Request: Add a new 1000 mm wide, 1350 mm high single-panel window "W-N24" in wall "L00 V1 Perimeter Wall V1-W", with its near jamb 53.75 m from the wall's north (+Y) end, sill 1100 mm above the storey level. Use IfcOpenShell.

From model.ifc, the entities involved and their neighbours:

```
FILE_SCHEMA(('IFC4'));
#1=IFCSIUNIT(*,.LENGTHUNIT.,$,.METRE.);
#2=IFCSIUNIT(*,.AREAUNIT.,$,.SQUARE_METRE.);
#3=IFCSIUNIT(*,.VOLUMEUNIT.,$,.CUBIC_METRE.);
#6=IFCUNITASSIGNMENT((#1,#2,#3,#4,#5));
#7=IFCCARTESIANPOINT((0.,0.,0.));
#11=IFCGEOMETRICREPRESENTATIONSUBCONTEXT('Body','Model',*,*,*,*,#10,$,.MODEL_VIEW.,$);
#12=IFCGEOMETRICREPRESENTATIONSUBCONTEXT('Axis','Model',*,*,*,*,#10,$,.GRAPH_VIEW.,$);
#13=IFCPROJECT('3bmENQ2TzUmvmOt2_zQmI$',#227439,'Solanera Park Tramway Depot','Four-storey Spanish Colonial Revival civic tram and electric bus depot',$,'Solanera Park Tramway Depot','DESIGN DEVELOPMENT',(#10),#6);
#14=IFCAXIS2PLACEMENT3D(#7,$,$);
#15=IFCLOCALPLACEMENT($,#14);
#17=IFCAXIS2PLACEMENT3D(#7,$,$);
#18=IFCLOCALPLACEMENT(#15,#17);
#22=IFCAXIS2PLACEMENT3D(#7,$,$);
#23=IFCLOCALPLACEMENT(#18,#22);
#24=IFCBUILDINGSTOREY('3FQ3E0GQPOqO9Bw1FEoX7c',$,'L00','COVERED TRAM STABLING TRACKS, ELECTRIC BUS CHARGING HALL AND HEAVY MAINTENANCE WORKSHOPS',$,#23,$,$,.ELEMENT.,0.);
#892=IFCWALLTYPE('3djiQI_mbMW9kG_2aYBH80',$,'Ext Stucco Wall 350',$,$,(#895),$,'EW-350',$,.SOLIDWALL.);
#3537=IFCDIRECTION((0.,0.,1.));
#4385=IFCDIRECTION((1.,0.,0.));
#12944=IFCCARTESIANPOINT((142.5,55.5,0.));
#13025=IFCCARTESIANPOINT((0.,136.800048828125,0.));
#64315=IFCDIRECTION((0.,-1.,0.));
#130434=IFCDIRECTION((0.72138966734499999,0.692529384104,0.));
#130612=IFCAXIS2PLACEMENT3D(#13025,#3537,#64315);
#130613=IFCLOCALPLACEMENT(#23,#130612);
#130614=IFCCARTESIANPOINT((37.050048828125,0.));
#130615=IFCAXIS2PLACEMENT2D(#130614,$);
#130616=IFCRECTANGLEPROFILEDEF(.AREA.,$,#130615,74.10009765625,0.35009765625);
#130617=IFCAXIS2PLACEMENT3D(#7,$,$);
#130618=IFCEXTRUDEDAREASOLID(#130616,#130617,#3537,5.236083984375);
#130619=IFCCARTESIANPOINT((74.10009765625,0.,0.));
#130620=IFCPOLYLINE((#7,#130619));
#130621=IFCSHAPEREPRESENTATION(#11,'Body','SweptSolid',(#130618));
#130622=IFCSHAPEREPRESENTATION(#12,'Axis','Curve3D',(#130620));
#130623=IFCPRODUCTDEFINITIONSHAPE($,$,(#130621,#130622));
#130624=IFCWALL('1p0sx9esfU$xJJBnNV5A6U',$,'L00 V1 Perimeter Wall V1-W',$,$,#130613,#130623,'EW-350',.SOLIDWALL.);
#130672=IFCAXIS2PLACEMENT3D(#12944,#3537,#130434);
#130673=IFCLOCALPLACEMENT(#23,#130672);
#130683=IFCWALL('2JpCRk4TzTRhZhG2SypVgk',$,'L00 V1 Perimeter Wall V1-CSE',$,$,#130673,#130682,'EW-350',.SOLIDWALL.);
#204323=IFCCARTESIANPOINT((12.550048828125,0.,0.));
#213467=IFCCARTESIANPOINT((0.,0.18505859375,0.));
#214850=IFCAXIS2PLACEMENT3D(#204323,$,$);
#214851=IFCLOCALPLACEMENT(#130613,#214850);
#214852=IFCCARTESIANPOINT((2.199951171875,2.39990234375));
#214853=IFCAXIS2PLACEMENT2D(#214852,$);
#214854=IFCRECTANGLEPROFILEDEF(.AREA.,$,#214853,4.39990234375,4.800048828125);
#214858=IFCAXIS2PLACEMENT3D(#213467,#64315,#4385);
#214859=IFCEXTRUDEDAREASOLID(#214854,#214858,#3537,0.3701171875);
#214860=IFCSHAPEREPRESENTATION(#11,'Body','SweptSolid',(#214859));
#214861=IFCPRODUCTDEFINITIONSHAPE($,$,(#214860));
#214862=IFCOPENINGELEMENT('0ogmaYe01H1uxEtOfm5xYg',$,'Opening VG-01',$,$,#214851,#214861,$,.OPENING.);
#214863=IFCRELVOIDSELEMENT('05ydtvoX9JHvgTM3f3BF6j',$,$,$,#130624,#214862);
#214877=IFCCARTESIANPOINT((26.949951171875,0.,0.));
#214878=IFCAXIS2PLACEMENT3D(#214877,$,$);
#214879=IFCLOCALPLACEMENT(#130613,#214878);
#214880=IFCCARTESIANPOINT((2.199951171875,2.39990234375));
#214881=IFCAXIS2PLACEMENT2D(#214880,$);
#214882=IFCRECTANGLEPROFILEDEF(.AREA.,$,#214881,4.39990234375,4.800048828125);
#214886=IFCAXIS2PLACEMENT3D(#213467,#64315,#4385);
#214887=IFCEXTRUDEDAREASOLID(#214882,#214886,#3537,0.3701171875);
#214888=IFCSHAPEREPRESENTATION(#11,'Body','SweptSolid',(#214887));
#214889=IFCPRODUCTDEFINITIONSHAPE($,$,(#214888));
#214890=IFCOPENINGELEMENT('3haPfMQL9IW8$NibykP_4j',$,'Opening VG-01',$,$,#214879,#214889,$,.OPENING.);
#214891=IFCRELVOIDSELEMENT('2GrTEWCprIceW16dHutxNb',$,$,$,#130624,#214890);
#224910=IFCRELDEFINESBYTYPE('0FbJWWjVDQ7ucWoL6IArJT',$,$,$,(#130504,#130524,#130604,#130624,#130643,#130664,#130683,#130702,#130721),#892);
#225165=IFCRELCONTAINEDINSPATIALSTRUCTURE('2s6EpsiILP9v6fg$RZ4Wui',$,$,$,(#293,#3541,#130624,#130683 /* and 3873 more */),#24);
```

```python
import numpy as np
import ifcopenshell
import ifcopenshell.api.feature
import ifcopenshell.api.geometry
import ifcopenshell.api.root
import ifcopenshell.api.spatial
import ifcopenshell.geom
import ifcopenshell.util.element
import ifcopenshell.util.placement
import ifcopenshell.util.representation
import ifcopenshell.util.shape
import ifcopenshell.util.unit

model = ifcopenshell.open("model.ifc")
unit_scale = ifcopenshell.util.unit.calculate_unit_scale(model)
settings = ifcopenshell.geom.settings()


def volume(element):
    """Net volume in cubic metres, openings subtracted."""
    shape = ifcopenshell.geom.create_shape(settings, element)
    return ifcopenshell.util.shape.get_volume(shape.geometry)


wall = model.by_guid("1p0sx9esfU$xJJBnNV5A6U")
storey = ifcopenshell.util.element.get_container(wall, ifc_class="IfcBuildingStorey")
context = ifcopenshell.util.representation.get_context(model, "Model", "Body", "MODEL_VIEW")
before = volume(wall)

width, height, from_end, sill = 1, 1.35, 53.75, 1.1  # metres

# The wall runs along its own X axis, and the end named is its -X end.
wall_shape = ifcopenshell.geom.create_shape(settings, wall)
x, y, z = ifcopenshell.util.shape.get_vertices(wall_shape.geometry).T
start = x.min() + from_end
face, thickness = float(y.min()), float(y.max() - y.min())
wall_matrix = ifcopenshell.util.placement.get_local_placement(wall.ObjectPlacement)
level = ifcopenshell.util.placement.get_local_placement(storey.ObjectPlacement)[2, 3]


def in_wall(x, y):
    """Placement at x, y metres in the wall's axes, at sill height."""
    matrix = wall_matrix.copy()
    matrix[:, 3] = wall_matrix @ np.array([x / unit_scale, y / unit_scale, 0.0, 1.0])
    matrix[2, 3] = level + sill / unit_scale
    return matrix


# Opening: a box that overshoots both wall faces by 50 mm.
opening = ifcopenshell.api.root.create_entity(model, ifc_class="IfcOpeningElement", predefined_type="OPENING")
box = ifcopenshell.api.geometry.add_wall_representation(
    model, context=context, length=width, height=height, thickness=thickness + 0.1
)
ifcopenshell.api.geometry.assign_representation(model, product=opening, representation=box)
ifcopenshell.api.geometry.edit_object_placement(model, product=opening, matrix=in_wall(start, face - 0.05), is_si=False)
ifcopenshell.api.feature.add_feature(model, feature=opening, element=wall)

window = ifcopenshell.api.root.create_entity(model, ifc_class="IfcWindow", name="W-N24", predefined_type="WINDOW")
window.OverallWidth, window.OverallHeight = width / unit_scale, height / unit_scale
window.PartitioningType = "SINGLE_PANEL"
body = ifcopenshell.api.geometry.add_window_representation(
    model,
    context=context,
    overall_width=window.OverallWidth,
    overall_height=window.OverallHeight,
    partition_type="SINGLE_PANEL",
)
ifcopenshell.api.geometry.assign_representation(model, product=window, representation=body)
ifcopenshell.api.spatial.assign_container(model, products=[window], relating_structure=storey)
ifcopenshell.api.feature.add_filling(model, opening=opening, element=window)

# Centre the window in the wall's thickness.
ifcopenshell.api.geometry.edit_object_placement(model, product=window, matrix=in_wall(start, face), is_si=False)
window_shape = ifcopenshell.geom.create_shape(settings, window)
depth = ifcopenshell.util.shape.get_vertices(window_shape.geometry)[:, 1]
offset = face + thickness / 2 - (depth.min() + depth.max()) / 2
ifcopenshell.api.geometry.edit_object_placement(model, product=window, matrix=in_wall(start, offset), is_si=False)

after = volume(wall)

print(f"wall volume {before:.3f} -> {after:.3f} m3")

model.write("model_rev.ifc")
```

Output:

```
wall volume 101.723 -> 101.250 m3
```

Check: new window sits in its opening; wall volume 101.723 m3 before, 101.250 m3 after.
